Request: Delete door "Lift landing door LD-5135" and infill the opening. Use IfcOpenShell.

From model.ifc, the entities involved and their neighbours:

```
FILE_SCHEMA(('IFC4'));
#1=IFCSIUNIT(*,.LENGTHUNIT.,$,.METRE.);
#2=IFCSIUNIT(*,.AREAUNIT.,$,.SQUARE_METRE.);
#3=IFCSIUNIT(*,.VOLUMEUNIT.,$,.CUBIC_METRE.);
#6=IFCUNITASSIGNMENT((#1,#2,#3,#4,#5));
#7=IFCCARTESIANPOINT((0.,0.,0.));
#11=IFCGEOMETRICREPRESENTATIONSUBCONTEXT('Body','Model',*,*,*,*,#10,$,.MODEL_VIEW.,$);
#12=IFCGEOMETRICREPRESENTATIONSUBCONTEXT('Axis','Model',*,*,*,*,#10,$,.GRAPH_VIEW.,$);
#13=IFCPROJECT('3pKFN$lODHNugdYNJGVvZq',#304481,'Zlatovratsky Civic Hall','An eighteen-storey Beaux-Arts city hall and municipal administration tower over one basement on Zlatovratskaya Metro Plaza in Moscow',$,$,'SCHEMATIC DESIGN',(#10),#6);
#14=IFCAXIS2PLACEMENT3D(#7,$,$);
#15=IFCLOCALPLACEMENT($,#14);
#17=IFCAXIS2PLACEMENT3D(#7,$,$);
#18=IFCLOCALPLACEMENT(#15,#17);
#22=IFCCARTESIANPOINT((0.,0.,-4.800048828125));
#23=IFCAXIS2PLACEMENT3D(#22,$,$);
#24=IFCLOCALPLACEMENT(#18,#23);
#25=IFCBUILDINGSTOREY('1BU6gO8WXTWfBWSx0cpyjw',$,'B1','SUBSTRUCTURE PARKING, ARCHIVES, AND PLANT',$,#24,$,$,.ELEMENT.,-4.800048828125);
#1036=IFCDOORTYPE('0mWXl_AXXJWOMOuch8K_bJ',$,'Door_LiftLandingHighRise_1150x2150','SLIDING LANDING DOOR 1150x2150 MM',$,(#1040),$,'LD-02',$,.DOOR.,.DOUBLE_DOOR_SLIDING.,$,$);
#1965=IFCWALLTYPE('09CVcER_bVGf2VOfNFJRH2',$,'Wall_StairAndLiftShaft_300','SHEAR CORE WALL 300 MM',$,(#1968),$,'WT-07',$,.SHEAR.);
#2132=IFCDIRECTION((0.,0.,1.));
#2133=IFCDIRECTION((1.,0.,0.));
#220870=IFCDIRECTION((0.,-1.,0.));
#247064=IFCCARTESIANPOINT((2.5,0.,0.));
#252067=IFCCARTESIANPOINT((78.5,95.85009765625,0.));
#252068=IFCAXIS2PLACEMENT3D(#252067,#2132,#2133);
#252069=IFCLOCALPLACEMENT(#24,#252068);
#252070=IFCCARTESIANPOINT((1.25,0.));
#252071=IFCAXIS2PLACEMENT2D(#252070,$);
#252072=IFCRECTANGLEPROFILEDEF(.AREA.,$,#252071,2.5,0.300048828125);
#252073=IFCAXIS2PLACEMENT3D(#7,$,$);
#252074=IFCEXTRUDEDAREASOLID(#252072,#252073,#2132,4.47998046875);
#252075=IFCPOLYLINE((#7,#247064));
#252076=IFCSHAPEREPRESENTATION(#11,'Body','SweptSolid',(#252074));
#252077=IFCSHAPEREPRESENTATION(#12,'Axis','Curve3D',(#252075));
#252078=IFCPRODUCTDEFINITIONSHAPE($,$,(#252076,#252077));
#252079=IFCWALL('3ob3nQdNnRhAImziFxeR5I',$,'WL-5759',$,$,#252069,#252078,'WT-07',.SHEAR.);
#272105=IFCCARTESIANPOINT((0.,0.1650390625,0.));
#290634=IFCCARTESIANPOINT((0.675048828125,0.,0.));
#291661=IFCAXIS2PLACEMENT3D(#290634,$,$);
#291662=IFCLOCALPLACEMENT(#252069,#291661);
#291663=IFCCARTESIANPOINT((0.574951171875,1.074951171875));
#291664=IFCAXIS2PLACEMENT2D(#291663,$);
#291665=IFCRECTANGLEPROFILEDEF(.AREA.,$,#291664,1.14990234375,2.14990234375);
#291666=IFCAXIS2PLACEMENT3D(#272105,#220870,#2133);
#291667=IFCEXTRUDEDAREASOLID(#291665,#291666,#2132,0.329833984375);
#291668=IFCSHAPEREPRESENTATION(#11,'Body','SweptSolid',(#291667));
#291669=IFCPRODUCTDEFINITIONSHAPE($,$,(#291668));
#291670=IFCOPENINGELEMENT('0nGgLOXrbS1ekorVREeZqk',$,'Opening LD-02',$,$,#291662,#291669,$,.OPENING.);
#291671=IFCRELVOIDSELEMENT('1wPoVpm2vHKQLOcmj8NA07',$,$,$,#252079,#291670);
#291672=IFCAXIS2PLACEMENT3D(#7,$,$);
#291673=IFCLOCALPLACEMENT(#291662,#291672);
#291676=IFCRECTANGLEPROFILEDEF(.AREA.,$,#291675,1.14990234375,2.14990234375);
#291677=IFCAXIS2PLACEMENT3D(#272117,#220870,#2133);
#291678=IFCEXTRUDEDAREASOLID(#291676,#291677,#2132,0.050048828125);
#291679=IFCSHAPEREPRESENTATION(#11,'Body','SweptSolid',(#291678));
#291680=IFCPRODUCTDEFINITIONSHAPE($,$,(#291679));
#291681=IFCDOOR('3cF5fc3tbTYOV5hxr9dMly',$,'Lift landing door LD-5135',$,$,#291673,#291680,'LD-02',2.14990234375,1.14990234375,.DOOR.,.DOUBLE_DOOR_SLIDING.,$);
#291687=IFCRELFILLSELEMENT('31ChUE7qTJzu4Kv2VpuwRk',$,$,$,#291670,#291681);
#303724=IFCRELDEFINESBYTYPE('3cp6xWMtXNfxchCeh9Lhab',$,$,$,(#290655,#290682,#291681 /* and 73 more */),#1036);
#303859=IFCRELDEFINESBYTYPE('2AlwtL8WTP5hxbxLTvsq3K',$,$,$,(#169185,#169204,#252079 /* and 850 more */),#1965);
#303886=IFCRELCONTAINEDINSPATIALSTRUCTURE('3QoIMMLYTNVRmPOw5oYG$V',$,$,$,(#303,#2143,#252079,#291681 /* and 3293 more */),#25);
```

```python
import ifcopenshell
import ifcopenshell.api.feature
import ifcopenshell.api.root
import ifcopenshell.geom
import ifcopenshell.util.shape

model = ifcopenshell.open("model.ifc")
settings = ifcopenshell.geom.settings()


def volume(element):
    """Net volume in cubic metres, openings subtracted."""
    shape = ifcopenshell.geom.create_shape(settings, element)
    return ifcopenshell.util.shape.get_volume(shape.geometry)


door = model.by_guid("3cF5fc3tbTYOV5hxr9dMly")
opening = door.FillsVoids[0].RelatingOpeningElement
wall = opening.VoidsElements[0].RelatingBuildingElement
before = volume(wall)

ifcopenshell.api.root.remove_product(model, product=door)
ifcopenshell.api.feature.remove_feature(model, feature=opening)

after = volume(wall)

print(f"wall volume {before:.3f} -> {after:.3f} m3")

model.write("model-out.ifc")
```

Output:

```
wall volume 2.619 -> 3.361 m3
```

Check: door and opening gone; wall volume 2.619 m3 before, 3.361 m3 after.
